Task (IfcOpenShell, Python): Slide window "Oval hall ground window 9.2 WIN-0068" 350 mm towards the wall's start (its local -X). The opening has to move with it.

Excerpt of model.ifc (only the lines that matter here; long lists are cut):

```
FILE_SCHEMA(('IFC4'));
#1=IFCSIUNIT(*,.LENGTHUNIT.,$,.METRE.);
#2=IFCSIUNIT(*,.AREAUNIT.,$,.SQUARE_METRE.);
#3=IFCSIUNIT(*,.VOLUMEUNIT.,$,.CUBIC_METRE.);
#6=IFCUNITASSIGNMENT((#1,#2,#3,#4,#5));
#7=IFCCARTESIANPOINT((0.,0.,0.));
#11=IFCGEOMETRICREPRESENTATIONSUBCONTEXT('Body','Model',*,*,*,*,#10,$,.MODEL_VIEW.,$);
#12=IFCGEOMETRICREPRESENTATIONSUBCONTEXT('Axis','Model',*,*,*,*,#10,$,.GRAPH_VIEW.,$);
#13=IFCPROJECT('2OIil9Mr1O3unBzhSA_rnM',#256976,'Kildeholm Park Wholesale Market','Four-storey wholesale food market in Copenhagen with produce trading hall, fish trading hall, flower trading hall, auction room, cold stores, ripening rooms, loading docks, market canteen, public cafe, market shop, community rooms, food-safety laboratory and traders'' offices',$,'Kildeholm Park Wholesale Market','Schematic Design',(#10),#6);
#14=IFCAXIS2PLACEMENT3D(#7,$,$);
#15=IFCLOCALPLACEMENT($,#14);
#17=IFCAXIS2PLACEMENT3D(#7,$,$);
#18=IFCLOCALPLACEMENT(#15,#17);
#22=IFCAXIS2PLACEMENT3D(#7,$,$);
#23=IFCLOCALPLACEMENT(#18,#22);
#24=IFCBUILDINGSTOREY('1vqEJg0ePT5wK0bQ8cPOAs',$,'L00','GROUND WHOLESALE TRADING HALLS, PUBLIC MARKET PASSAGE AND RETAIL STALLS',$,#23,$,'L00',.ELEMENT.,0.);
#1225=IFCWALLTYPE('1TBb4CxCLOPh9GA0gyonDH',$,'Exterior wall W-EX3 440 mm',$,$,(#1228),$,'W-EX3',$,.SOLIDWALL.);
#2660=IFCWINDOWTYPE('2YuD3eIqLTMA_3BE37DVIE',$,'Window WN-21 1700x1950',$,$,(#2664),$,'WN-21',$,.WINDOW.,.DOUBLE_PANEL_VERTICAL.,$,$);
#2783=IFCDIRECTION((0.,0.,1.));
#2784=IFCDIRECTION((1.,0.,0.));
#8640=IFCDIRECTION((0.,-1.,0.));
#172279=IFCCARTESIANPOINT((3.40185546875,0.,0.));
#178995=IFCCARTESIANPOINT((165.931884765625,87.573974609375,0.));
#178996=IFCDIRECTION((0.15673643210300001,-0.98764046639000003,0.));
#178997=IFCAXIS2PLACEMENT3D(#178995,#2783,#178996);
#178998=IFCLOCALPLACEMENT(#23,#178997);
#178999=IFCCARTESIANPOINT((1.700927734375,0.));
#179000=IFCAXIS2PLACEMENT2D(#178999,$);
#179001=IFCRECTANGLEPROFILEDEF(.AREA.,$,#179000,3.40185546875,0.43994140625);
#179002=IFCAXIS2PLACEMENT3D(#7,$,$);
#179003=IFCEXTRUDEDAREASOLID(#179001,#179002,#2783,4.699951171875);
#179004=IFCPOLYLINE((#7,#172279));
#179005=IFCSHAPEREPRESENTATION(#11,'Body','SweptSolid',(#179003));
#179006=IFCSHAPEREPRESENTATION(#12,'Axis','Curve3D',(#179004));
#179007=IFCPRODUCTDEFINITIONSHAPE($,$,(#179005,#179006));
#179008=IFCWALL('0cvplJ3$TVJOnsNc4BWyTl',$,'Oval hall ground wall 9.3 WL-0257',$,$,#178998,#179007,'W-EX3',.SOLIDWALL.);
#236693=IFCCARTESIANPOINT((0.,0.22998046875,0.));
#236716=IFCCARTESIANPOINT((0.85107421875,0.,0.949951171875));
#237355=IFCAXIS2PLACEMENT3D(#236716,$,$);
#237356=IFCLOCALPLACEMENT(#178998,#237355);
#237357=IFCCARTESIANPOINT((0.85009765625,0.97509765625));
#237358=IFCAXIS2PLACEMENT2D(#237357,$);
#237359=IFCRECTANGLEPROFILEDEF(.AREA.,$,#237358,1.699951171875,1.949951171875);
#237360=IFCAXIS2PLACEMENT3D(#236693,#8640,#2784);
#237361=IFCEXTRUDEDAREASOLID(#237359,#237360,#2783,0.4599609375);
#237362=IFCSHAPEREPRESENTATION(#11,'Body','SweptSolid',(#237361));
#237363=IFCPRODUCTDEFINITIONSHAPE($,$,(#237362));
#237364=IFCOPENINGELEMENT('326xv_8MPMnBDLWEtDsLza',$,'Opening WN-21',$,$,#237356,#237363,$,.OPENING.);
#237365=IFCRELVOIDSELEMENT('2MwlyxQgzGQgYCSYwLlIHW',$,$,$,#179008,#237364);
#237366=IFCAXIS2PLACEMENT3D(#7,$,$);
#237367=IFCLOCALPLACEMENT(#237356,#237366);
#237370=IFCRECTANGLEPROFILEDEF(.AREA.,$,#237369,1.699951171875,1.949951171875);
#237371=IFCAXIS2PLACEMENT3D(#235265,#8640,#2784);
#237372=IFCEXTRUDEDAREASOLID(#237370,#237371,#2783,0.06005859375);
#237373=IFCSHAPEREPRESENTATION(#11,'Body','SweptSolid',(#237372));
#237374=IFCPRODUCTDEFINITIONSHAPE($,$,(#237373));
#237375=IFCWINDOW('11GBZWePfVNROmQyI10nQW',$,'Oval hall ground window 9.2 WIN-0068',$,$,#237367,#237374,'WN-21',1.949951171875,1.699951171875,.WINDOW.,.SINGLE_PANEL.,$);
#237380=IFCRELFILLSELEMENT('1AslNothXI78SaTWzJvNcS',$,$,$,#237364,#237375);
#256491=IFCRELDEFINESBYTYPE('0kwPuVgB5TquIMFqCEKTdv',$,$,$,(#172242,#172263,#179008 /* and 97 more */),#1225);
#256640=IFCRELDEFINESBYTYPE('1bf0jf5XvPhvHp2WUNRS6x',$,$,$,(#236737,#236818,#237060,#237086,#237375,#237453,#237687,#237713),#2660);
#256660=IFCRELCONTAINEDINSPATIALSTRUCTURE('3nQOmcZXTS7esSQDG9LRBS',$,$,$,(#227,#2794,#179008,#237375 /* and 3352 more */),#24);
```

```python
import ifcopenshell
import ifcopenshell.api.geometry
import ifcopenshell.util.placement
import ifcopenshell.util.unit

model = ifcopenshell.open("model.ifc")
unit_scale = ifcopenshell.util.unit.calculate_unit_scale(model)

window = model.by_guid("11GBZWePfVNROmQyI10nQW")
opening = window.FillsVoids[0].RelatingOpeningElement
wall = opening.VoidsElements[0].RelatingBuildingElement

wall_matrix = ifcopenshell.util.placement.get_local_placement(wall.ObjectPlacement)
shift = wall_matrix[:3, 0] * -0.35 / unit_scale
before = ifcopenshell.util.placement.get_local_placement(window.ObjectPlacement)[:3, 3].copy()

# The window is placed relative to its opening, so it follows when the opening moves.
matrix = ifcopenshell.util.placement.get_local_placement(opening.ObjectPlacement)
matrix[:3, 3] += shift
ifcopenshell.api.geometry.edit_object_placement(
    model, product=opening, matrix=matrix, is_si=False, should_transform_children=True
)

after = ifcopenshell.util.placement.get_local_placement(window.ObjectPlacement)[:3, 3]
print("window moved by", (after - before).round(3) + 0.0)

model.write("model_updated.ifc")
```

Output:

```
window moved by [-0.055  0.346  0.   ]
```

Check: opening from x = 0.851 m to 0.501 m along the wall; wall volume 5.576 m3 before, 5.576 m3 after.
